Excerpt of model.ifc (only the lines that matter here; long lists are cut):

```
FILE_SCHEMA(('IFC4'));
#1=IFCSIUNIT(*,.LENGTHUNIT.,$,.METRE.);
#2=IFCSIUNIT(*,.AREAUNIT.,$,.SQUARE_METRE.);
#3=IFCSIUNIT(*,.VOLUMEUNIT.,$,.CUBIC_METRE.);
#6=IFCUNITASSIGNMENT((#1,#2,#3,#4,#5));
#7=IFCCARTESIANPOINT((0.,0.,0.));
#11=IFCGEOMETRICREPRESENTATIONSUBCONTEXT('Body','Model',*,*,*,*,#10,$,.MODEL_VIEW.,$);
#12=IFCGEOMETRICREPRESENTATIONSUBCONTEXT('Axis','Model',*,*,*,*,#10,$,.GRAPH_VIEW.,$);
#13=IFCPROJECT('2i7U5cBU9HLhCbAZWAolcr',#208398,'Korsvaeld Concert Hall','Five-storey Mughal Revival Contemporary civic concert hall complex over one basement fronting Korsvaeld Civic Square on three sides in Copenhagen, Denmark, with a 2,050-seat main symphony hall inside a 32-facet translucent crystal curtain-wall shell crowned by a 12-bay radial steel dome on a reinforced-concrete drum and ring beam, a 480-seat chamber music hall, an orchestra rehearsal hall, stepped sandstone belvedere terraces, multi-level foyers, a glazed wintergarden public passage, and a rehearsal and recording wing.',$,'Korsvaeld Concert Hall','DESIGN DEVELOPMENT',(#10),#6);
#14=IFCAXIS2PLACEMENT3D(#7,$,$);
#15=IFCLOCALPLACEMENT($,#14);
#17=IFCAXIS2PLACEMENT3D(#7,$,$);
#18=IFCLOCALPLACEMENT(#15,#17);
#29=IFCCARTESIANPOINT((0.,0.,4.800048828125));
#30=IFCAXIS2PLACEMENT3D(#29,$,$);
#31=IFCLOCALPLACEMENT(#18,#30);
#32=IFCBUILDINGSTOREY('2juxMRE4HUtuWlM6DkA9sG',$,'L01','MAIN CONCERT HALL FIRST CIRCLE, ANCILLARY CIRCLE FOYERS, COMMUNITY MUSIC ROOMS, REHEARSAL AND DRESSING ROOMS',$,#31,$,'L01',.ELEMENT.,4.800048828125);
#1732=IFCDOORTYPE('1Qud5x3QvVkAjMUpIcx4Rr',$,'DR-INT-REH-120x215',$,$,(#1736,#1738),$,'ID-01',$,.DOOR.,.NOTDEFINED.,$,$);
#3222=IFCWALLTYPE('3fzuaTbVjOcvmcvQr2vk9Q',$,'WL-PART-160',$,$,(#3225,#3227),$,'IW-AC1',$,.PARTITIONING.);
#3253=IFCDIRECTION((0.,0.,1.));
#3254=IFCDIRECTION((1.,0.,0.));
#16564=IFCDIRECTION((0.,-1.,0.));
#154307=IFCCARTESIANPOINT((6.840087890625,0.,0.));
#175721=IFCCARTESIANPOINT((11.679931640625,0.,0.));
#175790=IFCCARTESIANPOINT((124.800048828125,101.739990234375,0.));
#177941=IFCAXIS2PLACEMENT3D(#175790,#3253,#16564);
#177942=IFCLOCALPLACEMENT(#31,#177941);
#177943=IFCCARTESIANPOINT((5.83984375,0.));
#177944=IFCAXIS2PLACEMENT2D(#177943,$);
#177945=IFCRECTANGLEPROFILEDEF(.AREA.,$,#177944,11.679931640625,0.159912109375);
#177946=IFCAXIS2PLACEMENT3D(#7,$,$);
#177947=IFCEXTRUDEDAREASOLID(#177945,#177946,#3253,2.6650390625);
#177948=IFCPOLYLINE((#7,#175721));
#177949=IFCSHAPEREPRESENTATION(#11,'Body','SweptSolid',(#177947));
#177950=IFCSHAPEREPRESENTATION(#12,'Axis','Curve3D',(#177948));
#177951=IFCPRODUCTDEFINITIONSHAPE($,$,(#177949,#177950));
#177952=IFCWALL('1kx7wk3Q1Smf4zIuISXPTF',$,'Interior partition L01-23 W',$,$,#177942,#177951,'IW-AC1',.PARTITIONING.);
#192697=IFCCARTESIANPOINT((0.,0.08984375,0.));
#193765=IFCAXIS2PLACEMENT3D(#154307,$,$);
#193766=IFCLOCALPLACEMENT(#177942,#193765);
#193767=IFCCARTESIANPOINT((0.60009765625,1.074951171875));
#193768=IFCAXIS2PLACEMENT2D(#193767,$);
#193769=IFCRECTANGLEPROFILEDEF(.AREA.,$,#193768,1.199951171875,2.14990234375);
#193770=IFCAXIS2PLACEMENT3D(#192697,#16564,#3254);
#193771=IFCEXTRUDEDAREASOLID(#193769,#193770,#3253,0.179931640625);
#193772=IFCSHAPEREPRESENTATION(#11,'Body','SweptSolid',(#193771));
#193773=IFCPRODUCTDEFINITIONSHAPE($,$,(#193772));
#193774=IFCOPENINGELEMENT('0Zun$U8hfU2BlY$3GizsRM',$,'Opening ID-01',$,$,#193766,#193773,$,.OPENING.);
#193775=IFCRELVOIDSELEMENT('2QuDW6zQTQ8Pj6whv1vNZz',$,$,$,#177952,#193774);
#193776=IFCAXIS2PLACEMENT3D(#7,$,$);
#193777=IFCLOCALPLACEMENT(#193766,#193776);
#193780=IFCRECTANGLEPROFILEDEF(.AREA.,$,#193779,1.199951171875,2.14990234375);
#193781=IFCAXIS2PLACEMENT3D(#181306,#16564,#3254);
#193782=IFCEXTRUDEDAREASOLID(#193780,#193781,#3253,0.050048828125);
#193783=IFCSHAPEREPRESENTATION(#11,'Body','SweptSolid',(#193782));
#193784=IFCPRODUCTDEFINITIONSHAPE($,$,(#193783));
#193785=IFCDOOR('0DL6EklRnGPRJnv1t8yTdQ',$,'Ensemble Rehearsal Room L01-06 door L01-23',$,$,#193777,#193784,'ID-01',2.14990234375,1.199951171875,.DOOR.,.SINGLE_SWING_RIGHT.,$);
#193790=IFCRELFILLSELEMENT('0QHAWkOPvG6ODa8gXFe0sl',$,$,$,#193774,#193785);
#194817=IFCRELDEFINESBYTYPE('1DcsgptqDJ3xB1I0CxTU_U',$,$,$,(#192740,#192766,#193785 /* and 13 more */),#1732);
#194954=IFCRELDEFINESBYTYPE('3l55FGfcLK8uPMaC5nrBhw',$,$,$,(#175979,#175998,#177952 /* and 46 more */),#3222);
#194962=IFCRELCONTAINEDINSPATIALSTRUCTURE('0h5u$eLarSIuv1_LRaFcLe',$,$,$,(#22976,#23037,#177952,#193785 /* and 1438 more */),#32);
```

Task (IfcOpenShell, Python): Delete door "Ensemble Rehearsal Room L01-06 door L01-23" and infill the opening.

```python
import ifcopenshell
import ifcopenshell.api.feature
import ifcopenshell.api.root
import ifcopenshell.geom
import ifcopenshell.util.shape

model = ifcopenshell.open("model.ifc")
settings = ifcopenshell.geom.settings()


def volume(element):
    """Net volume in cubic metres, openings subtracted."""
    shape = ifcopenshell.geom.create_shape(settings, element)
    return ifcopenshell.util.shape.get_volume(shape.geometry)


door = model.by_guid("0DL6EklRnGPRJnv1t8yTdQ")
opening = door.FillsVoids[0].RelatingOpeningElement
wall = opening.VoidsElements[0].RelatingBuildingElement
before = volume(wall)

ifcopenshell.api.root.remove_product(model, product=door)
ifcopenshell.api.feature.remove_feature(model, feature=opening)

after = volume(wall)

print(f"wall volume {before:.3f} -> {after:.3f} m3")

model.write("model-out.ifc")
```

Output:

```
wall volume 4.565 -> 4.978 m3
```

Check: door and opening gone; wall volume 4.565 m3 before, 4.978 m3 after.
